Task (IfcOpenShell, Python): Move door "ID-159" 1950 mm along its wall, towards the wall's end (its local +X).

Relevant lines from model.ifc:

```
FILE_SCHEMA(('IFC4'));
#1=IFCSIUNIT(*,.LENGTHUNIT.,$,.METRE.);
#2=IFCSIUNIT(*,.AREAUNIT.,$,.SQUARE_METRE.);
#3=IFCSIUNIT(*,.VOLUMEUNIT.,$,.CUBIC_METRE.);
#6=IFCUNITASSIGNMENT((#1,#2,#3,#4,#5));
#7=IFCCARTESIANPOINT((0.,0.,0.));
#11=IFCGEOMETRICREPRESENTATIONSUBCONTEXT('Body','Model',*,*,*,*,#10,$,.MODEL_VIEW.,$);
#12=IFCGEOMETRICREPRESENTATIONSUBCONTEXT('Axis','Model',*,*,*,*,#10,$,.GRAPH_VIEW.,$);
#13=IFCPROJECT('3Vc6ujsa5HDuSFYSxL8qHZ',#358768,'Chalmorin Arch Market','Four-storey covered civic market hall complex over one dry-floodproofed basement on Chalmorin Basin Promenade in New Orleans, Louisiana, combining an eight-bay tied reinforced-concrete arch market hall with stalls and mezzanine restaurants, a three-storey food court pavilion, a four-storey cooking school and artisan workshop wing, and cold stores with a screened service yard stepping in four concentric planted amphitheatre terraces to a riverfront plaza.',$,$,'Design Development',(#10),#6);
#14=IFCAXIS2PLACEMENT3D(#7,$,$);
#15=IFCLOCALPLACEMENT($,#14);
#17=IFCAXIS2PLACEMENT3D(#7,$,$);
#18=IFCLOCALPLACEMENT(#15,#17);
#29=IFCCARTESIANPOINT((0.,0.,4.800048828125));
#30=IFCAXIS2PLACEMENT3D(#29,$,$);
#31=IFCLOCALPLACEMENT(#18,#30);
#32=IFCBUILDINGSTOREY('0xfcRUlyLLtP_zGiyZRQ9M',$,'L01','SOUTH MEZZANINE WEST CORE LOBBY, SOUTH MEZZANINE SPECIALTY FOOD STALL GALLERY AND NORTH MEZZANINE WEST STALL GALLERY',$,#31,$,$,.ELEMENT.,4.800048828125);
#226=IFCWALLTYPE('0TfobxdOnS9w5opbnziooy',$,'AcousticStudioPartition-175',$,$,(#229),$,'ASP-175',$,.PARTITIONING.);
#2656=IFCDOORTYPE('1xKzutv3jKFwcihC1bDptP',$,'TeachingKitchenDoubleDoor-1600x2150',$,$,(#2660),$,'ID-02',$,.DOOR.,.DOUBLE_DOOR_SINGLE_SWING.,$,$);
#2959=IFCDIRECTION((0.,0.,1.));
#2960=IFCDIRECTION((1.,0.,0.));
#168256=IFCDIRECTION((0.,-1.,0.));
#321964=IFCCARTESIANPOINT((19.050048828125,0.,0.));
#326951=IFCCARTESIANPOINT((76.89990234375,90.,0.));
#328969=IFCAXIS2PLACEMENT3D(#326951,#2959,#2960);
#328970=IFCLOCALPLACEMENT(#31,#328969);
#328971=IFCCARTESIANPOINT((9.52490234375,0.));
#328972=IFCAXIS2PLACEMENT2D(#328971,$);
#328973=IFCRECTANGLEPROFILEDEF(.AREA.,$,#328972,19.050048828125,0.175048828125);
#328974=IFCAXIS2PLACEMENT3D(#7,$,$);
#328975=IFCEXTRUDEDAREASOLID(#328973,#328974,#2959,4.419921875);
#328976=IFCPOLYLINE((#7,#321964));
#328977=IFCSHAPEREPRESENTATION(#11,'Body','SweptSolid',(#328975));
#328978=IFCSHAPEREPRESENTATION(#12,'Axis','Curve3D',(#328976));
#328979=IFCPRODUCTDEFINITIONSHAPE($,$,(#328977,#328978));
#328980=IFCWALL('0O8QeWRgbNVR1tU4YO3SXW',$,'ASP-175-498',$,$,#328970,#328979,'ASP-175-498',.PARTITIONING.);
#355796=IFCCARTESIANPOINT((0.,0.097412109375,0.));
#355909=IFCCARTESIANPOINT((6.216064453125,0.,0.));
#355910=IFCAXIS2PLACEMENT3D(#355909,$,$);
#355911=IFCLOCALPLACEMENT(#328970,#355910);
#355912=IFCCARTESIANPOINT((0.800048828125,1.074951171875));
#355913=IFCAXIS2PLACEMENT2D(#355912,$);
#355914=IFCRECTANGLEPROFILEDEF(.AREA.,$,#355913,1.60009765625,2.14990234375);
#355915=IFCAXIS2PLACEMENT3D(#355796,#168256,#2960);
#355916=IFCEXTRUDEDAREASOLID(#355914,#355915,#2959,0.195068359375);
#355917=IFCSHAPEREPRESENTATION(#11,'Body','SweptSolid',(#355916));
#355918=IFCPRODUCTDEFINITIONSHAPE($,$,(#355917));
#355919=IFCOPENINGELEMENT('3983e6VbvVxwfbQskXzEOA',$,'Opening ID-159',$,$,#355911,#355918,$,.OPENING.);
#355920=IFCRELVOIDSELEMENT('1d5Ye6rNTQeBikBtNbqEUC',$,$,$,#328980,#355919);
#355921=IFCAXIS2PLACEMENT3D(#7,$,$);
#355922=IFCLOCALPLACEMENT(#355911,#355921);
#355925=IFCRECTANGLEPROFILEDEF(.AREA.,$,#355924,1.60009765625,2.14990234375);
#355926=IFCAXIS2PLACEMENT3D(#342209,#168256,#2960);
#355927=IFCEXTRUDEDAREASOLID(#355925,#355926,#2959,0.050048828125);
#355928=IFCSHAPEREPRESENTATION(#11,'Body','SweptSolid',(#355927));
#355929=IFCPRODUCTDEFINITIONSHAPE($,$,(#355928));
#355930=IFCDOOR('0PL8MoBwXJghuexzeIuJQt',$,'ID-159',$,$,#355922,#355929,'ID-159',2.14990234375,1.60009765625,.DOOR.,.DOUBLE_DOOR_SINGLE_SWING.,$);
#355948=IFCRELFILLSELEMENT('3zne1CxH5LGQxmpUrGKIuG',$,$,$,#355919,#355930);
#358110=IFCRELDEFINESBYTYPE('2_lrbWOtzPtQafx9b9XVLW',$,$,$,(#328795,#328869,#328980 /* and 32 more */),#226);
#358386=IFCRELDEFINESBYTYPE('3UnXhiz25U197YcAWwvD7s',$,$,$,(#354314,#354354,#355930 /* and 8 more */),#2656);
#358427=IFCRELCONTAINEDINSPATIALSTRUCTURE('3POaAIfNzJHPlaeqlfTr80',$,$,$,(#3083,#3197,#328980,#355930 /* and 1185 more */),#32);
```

```python
import ifcopenshell
import ifcopenshell.api.geometry
import ifcopenshell.util.placement
import ifcopenshell.util.unit

model = ifcopenshell.open("model.ifc")
unit_scale = ifcopenshell.util.unit.calculate_unit_scale(model)

door = model.by_guid("0PL8MoBwXJghuexzeIuJQt")
opening = door.FillsVoids[0].RelatingOpeningElement
wall = opening.VoidsElements[0].RelatingBuildingElement

wall_matrix = ifcopenshell.util.placement.get_local_placement(wall.ObjectPlacement)
shift = wall_matrix[:3, 0] * 1.95 / unit_scale
before = ifcopenshell.util.placement.get_local_placement(door.ObjectPlacement)[:3, 3].copy()

# The door is placed relative to its opening, so it follows when the opening moves.
matrix = ifcopenshell.util.placement.get_local_placement(opening.ObjectPlacement)
matrix[:3, 3] += shift
ifcopenshell.api.geometry.edit_object_placement(
    model, product=opening, matrix=matrix, is_si=False, should_transform_children=True
)

after = ifcopenshell.util.placement.get_local_placement(door.ObjectPlacement)[:3, 3]
print("door moved by", (after - before).round(3) + 0.0)

model.write("model_edited.ifc")
```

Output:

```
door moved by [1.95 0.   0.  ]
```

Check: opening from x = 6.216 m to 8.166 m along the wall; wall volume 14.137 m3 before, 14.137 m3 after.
